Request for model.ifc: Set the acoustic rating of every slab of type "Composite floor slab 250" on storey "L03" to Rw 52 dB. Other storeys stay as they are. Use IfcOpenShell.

First a look at what the model holds.

```python
import ifcopenshell
import ifcopenshell.util.element

model = ifcopenshell.open("model.ifc")
print(model.schema)
storey = next(s for s in model.by_type("IfcBuildingStorey") if s.Name == "L03")
slabs = [e for e in ifcopenshell.util.element.get_decomposition(storey) if e.is_a("IfcSlab")]
seen = {}
for e in slabs:
    element_type = ifcopenshell.util.element.get_type(e)
    key = (element_type.Name if element_type != e and element_type else None, ifcopenshell.util.element.get_pset(e, "Pset_SlabCommon", "AcousticRating"))
    seen[key] = seen.get(key, 0) + 1
for (name, value), count in sorted(seen.items(), key=str):
    print(count, "x", name, "|", value)
```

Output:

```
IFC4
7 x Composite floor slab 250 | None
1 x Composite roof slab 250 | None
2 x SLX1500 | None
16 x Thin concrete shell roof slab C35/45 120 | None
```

```python
import ifcopenshell
import ifcopenshell.api.pset
import ifcopenshell.util.element

model = ifcopenshell.open("model.ifc")

storey = next(s for s in model.by_type("IfcBuildingStorey") if s.Name == "L03")
slabs = [e for e in ifcopenshell.util.element.get_decomposition(storey) if e.is_a("IfcSlab")]

count = 0
for e in slabs:
    element_type = ifcopenshell.util.element.get_type(e)
    if element_type in (None, e) or element_type.Name != "Composite floor slab 250":
        continue
    # add_pset returns the element's existing set when there is one.
    pset = ifcopenshell.api.pset.add_pset(model, product=e, name="Pset_SlabCommon")
    ifcopenshell.api.pset.edit_pset(model, pset=pset, properties={"AcousticRating": "Rw 52 dB"})
    count += 1

print(count, "slabs updated")

model.write("model_rev.ifc")
```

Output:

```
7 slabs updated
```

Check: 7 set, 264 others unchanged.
